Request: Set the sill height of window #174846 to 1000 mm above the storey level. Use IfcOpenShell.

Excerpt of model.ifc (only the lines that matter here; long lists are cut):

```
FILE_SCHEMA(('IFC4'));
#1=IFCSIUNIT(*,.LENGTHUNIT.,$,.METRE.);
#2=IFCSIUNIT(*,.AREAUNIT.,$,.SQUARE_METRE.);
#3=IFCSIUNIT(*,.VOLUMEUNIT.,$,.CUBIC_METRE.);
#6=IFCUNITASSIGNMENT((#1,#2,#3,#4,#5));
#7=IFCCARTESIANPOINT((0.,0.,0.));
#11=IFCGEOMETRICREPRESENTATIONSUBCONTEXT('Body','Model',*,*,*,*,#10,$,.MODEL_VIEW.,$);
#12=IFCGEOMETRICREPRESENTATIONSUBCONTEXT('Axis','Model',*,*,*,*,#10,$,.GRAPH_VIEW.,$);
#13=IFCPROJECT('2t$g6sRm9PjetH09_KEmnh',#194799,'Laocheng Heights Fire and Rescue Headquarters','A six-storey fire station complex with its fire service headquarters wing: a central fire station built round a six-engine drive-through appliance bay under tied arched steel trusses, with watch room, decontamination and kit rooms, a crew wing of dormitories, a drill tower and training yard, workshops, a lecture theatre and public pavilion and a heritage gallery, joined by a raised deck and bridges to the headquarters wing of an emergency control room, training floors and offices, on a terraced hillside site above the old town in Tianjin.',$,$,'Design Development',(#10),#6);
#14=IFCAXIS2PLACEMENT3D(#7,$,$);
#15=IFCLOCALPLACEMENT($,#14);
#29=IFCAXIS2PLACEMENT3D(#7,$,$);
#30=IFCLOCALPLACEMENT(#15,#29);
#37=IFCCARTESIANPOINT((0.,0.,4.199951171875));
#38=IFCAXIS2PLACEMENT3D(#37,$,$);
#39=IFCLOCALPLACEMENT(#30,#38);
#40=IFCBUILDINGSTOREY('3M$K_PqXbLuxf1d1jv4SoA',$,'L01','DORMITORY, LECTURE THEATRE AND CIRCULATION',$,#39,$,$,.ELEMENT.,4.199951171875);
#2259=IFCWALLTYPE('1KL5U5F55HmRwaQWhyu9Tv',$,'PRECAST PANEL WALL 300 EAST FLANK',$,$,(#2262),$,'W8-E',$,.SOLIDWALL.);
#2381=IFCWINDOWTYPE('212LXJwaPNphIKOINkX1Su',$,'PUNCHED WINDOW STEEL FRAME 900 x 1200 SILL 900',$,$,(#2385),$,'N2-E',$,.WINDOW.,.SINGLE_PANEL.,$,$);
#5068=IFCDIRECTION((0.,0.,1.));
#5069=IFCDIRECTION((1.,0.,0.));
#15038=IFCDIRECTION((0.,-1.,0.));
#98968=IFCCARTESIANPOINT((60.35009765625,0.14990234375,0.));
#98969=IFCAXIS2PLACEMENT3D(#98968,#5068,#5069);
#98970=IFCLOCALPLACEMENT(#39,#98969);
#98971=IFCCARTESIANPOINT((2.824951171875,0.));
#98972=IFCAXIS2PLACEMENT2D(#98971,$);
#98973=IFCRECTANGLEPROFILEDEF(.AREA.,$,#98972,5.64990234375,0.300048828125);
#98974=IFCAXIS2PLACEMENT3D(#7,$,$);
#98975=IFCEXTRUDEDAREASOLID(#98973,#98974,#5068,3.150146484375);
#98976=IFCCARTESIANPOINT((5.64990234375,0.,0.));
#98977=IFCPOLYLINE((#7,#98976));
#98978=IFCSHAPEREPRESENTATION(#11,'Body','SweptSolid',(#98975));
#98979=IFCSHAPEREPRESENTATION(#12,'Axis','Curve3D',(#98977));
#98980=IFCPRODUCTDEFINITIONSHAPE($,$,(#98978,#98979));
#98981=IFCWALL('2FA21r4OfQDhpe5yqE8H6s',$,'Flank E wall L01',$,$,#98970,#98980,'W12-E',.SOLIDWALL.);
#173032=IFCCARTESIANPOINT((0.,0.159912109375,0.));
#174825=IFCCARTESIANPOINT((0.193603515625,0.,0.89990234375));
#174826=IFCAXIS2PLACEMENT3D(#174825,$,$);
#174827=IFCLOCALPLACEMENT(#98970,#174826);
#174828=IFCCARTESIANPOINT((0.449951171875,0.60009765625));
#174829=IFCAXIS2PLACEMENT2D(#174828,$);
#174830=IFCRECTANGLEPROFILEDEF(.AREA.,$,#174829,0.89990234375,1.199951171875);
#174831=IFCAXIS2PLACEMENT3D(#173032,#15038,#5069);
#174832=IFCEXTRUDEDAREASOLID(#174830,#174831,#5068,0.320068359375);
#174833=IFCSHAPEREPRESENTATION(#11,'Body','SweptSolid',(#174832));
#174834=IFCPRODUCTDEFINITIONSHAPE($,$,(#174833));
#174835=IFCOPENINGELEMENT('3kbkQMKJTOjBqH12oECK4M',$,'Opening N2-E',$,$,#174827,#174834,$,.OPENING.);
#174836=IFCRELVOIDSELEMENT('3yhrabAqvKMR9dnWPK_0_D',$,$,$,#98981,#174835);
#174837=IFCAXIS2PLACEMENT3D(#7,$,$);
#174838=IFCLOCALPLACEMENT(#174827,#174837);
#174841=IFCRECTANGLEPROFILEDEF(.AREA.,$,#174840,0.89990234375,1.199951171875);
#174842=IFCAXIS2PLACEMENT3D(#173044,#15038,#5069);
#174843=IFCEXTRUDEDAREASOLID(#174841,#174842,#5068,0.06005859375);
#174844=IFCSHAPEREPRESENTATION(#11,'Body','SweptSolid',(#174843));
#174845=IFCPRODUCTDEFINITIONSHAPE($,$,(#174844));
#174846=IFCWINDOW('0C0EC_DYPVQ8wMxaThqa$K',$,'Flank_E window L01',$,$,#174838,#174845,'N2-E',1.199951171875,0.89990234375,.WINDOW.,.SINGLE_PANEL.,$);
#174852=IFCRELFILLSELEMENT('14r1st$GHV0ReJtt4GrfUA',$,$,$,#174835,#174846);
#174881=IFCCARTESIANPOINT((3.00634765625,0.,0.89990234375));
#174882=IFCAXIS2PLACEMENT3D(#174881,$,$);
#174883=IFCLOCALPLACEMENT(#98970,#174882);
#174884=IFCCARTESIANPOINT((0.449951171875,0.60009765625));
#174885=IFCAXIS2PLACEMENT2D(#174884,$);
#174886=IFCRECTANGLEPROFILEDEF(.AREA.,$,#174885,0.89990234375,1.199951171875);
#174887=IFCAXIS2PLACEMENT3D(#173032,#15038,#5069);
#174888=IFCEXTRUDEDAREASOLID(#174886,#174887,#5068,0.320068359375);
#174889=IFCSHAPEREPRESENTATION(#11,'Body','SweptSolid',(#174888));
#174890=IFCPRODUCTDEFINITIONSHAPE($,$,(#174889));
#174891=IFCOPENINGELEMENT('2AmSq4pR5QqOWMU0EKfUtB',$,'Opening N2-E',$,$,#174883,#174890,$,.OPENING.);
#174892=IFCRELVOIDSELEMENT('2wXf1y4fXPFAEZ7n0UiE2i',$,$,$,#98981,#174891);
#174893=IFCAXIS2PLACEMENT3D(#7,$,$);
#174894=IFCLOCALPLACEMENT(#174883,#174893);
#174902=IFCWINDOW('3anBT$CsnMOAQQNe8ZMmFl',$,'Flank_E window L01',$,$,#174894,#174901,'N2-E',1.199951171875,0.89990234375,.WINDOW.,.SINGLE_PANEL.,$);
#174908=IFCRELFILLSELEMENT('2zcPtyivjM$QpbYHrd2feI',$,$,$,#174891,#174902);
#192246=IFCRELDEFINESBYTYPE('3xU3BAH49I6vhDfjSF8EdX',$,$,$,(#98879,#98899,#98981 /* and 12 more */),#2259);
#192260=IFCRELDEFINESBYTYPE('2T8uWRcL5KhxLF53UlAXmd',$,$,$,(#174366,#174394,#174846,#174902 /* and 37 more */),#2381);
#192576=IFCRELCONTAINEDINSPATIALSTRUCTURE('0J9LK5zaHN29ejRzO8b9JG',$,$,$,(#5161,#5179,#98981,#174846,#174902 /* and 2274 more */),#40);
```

```python
import numpy as np
import ifcopenshell
import ifcopenshell.api.geometry
import ifcopenshell.geom
import ifcopenshell.util.element
import ifcopenshell.util.placement
import ifcopenshell.util.shape
import ifcopenshell.util.unit

model = ifcopenshell.open("model.ifc")
unit_scale = ifcopenshell.util.unit.calculate_unit_scale(model)

window = model.by_id(174846)
opening = window.FillsVoids[0].RelatingOpeningElement
storey = ifcopenshell.util.element.get_container(window, ifc_class="IfcBuildingStorey")
level = ifcopenshell.util.placement.get_local_placement(storey.ObjectPlacement)[2, 3]

# The opening's origin need not be at the sill, so measure its lowest point.
shape = ifcopenshell.geom.create_shape(ifcopenshell.geom.settings(), opening)
bottom = ifcopenshell.util.shape.get_shape_bottom_elevation(shape, shape.geometry) / unit_scale
dz = level + 1 / unit_scale - bottom

shift = np.array([0.0, 0.0, dz])
# The window is placed relative to its opening, so it follows when the opening moves.
matrix = ifcopenshell.util.placement.get_local_placement(opening.ObjectPlacement)
matrix[:3, 3] += shift
ifcopenshell.api.geometry.edit_object_placement(
    model, product=opening, matrix=matrix, is_si=False, should_transform_children=True
)

print(f"moved by {dz * unit_scale:+.3f} m")

model.write("model_edited.ifc")
```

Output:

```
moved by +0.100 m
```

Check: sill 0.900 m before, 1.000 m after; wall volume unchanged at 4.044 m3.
